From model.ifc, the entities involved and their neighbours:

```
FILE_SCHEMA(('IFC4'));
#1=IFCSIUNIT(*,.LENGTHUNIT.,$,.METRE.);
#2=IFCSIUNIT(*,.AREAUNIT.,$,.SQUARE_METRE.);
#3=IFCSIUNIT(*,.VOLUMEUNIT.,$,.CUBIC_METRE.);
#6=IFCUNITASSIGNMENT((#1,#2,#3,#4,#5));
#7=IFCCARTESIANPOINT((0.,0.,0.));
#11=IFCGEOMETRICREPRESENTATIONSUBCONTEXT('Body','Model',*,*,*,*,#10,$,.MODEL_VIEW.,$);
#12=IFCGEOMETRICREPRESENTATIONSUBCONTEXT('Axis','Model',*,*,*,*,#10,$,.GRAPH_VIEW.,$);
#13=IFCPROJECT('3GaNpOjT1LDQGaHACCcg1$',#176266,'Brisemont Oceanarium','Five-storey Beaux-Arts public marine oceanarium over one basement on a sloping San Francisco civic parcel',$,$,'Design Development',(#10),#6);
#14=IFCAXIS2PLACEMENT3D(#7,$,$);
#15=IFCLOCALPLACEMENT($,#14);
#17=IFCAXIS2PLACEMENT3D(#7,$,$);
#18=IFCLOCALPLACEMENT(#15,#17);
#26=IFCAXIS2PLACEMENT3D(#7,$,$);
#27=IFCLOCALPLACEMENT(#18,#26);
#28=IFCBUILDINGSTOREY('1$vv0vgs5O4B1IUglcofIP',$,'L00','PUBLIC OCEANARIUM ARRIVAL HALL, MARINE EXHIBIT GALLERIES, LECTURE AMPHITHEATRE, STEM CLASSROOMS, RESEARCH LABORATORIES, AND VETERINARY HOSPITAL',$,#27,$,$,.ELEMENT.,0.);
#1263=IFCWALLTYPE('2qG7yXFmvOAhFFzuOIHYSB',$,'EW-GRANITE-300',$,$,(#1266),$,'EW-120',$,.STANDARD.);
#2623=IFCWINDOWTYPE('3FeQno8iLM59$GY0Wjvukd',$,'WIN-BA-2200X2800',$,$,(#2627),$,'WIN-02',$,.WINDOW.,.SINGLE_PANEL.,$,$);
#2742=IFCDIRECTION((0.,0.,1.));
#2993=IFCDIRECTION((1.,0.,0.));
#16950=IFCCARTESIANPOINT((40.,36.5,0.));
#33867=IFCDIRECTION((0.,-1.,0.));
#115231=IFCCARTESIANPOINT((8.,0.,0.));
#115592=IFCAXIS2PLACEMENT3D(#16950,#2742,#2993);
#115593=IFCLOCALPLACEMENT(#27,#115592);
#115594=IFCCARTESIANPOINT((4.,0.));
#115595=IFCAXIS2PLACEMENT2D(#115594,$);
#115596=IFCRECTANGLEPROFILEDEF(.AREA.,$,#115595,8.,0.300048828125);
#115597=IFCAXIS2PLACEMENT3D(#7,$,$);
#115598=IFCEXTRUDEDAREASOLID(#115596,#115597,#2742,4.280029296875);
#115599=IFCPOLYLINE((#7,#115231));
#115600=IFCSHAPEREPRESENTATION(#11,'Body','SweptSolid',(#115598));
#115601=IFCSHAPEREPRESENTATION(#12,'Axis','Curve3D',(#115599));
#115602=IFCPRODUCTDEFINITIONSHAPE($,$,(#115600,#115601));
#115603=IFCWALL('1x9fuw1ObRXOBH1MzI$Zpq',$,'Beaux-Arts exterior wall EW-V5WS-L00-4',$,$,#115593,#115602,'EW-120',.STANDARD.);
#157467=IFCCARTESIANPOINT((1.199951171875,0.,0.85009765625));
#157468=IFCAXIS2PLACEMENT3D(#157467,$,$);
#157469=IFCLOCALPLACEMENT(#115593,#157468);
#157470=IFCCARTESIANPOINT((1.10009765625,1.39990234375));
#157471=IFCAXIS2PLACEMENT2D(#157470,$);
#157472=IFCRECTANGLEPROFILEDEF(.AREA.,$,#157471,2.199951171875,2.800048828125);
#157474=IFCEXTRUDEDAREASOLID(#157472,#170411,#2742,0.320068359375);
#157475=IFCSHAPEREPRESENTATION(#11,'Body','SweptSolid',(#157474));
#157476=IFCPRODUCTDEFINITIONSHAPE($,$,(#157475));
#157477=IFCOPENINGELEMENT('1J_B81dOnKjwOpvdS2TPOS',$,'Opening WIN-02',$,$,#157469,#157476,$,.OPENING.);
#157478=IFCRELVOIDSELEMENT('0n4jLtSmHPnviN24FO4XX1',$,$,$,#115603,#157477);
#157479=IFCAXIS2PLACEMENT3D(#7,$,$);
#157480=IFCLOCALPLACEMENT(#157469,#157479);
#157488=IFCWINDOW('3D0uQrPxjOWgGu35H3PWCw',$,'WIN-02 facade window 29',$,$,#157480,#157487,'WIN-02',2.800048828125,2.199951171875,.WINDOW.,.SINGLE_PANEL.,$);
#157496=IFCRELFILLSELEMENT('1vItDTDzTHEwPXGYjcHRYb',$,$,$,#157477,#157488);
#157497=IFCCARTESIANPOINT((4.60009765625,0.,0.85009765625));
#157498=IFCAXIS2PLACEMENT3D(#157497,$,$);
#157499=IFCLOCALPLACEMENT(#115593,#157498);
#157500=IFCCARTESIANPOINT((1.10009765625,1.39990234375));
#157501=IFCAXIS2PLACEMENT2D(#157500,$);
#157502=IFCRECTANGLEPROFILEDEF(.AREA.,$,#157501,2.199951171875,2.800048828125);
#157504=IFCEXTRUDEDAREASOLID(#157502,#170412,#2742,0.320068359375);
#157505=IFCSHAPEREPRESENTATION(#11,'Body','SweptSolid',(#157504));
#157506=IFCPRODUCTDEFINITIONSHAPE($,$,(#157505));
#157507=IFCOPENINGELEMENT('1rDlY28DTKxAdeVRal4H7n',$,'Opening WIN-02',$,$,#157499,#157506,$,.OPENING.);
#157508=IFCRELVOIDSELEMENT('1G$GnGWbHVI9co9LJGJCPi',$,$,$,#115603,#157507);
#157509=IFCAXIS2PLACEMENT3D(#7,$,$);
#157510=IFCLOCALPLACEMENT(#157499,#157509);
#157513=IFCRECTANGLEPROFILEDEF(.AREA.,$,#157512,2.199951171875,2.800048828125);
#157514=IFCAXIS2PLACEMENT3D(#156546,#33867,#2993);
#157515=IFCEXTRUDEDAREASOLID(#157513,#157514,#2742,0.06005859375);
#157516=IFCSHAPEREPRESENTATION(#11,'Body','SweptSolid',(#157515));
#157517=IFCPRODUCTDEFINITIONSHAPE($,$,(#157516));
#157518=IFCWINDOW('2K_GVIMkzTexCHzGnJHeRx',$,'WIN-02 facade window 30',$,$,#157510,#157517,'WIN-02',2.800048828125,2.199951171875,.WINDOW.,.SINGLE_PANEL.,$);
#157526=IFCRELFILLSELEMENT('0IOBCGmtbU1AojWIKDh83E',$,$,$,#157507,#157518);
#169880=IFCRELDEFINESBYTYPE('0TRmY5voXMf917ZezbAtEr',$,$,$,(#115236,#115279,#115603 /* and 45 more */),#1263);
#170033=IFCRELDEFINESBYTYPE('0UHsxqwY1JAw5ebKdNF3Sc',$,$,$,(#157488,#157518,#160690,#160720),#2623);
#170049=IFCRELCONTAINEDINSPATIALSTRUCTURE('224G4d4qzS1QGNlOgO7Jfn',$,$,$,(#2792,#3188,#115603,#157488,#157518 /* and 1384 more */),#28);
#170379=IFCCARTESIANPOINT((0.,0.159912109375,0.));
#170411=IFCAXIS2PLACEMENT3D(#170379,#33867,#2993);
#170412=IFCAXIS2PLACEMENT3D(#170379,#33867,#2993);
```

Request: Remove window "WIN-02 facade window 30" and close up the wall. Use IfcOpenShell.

```python
import ifcopenshell
import ifcopenshell.api.feature
import ifcopenshell.api.root
import ifcopenshell.geom
import ifcopenshell.util.shape

model = ifcopenshell.open("model.ifc")
settings = ifcopenshell.geom.settings()


def volume(element):
    """Net volume in cubic metres, openings subtracted."""
    shape = ifcopenshell.geom.create_shape(settings, element)
    return ifcopenshell.util.shape.get_volume(shape.geometry)


window = model.by_id(157518)
opening = window.FillsVoids[0].RelatingOpeningElement
wall = opening.VoidsElements[0].RelatingBuildingElement
before = volume(wall)

ifcopenshell.api.root.remove_product(model, product=window)
ifcopenshell.api.feature.remove_feature(model, feature=opening)

after = volume(wall)

print(f"wall volume {before:.3f} -> {after:.3f} m3")

model.write("model-out.ifc")
```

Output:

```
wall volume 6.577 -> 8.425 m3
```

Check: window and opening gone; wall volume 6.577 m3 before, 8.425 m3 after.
